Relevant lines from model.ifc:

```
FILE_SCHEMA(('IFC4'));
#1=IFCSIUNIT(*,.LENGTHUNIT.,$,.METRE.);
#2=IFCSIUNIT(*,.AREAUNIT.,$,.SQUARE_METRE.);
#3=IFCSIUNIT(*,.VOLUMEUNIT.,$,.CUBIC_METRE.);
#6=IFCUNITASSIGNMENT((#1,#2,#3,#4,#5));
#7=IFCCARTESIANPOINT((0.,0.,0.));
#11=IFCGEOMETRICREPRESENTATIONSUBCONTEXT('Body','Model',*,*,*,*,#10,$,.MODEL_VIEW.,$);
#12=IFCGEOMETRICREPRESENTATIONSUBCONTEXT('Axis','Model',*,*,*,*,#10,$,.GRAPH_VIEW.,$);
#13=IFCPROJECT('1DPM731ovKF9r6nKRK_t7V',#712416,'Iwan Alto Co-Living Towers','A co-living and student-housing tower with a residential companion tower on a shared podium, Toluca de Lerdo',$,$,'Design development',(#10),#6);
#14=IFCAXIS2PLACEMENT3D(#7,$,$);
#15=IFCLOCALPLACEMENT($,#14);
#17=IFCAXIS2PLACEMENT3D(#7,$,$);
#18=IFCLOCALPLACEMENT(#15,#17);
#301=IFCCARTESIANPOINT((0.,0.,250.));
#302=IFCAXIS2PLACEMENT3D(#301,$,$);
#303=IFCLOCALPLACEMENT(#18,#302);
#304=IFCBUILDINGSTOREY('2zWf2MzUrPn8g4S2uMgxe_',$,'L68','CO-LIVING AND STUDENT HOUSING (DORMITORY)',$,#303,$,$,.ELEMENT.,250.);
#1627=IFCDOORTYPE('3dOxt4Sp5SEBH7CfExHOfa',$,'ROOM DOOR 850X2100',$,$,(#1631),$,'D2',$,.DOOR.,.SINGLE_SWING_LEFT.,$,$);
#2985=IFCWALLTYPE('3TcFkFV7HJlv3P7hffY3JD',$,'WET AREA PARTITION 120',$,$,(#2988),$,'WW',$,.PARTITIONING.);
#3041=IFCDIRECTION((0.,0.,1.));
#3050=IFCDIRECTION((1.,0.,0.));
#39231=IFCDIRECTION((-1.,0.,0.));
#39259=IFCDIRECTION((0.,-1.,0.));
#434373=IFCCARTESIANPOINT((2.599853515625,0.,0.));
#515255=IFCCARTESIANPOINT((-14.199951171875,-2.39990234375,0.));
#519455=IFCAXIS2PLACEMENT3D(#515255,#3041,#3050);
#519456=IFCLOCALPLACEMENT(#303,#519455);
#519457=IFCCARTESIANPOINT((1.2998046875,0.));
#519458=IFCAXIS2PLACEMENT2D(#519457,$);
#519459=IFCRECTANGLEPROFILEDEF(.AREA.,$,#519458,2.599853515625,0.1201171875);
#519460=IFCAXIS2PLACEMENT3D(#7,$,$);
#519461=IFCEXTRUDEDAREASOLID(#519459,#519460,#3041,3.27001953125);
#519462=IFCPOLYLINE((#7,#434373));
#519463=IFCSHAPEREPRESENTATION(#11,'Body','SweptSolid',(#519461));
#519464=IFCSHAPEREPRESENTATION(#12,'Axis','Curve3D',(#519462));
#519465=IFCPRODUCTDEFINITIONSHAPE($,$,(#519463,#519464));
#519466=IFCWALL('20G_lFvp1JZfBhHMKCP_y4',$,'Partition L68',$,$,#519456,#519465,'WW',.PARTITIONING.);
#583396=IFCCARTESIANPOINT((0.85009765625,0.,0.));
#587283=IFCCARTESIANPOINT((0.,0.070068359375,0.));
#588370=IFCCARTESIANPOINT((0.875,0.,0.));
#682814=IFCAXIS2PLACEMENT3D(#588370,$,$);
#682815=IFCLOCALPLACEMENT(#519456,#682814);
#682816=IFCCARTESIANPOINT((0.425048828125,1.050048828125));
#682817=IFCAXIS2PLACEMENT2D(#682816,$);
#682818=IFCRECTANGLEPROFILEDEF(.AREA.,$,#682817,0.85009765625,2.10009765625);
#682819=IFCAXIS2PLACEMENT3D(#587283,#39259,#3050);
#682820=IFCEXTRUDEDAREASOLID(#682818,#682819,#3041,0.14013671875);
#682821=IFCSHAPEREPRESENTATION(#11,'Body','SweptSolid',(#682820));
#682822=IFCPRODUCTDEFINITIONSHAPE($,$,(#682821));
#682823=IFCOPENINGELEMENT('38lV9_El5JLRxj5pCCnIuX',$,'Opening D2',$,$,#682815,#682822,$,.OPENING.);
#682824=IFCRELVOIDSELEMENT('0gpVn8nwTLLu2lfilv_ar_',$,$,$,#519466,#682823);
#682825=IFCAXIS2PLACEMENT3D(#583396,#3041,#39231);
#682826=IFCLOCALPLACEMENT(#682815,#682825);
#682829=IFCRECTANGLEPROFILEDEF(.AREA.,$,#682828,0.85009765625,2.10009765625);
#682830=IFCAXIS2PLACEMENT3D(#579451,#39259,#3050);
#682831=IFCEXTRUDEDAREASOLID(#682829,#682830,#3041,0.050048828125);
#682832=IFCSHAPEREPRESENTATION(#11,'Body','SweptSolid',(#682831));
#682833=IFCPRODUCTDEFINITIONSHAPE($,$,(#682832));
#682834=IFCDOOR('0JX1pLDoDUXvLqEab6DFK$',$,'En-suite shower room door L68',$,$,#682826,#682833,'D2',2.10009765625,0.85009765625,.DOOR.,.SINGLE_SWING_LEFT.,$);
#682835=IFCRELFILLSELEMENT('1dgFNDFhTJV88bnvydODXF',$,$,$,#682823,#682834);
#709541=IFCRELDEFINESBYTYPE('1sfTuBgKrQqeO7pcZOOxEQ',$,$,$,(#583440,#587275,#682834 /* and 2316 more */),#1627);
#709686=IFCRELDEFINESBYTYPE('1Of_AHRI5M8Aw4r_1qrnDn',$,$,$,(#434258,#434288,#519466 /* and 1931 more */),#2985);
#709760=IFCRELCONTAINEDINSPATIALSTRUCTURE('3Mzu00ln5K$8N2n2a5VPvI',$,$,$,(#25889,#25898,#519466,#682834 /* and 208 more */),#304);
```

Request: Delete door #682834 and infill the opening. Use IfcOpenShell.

```python
import ifcopenshell
import ifcopenshell.api.feature
import ifcopenshell.api.root
import ifcopenshell.geom
import ifcopenshell.util.shape

model = ifcopenshell.open("model.ifc")
settings = ifcopenshell.geom.settings()


def volume(element):
    """Net volume in cubic metres, openings subtracted."""
    shape = ifcopenshell.geom.create_shape(settings, element)
    return ifcopenshell.util.shape.get_volume(shape.geometry)


door = model.by_guid("0JX1pLDoDUXvLqEab6DFK$")
opening = door.FillsVoids[0].RelatingOpeningElement
wall = opening.VoidsElements[0].RelatingBuildingElement
before = volume(wall)

ifcopenshell.api.root.remove_product(model, product=door)
ifcopenshell.api.feature.remove_feature(model, feature=opening)

after = volume(wall)

print(f"wall volume {before:.3f} -> {after:.3f} m3")

model.write("model_updated.ifc")
```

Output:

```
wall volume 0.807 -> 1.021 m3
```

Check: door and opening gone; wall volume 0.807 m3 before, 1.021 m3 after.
